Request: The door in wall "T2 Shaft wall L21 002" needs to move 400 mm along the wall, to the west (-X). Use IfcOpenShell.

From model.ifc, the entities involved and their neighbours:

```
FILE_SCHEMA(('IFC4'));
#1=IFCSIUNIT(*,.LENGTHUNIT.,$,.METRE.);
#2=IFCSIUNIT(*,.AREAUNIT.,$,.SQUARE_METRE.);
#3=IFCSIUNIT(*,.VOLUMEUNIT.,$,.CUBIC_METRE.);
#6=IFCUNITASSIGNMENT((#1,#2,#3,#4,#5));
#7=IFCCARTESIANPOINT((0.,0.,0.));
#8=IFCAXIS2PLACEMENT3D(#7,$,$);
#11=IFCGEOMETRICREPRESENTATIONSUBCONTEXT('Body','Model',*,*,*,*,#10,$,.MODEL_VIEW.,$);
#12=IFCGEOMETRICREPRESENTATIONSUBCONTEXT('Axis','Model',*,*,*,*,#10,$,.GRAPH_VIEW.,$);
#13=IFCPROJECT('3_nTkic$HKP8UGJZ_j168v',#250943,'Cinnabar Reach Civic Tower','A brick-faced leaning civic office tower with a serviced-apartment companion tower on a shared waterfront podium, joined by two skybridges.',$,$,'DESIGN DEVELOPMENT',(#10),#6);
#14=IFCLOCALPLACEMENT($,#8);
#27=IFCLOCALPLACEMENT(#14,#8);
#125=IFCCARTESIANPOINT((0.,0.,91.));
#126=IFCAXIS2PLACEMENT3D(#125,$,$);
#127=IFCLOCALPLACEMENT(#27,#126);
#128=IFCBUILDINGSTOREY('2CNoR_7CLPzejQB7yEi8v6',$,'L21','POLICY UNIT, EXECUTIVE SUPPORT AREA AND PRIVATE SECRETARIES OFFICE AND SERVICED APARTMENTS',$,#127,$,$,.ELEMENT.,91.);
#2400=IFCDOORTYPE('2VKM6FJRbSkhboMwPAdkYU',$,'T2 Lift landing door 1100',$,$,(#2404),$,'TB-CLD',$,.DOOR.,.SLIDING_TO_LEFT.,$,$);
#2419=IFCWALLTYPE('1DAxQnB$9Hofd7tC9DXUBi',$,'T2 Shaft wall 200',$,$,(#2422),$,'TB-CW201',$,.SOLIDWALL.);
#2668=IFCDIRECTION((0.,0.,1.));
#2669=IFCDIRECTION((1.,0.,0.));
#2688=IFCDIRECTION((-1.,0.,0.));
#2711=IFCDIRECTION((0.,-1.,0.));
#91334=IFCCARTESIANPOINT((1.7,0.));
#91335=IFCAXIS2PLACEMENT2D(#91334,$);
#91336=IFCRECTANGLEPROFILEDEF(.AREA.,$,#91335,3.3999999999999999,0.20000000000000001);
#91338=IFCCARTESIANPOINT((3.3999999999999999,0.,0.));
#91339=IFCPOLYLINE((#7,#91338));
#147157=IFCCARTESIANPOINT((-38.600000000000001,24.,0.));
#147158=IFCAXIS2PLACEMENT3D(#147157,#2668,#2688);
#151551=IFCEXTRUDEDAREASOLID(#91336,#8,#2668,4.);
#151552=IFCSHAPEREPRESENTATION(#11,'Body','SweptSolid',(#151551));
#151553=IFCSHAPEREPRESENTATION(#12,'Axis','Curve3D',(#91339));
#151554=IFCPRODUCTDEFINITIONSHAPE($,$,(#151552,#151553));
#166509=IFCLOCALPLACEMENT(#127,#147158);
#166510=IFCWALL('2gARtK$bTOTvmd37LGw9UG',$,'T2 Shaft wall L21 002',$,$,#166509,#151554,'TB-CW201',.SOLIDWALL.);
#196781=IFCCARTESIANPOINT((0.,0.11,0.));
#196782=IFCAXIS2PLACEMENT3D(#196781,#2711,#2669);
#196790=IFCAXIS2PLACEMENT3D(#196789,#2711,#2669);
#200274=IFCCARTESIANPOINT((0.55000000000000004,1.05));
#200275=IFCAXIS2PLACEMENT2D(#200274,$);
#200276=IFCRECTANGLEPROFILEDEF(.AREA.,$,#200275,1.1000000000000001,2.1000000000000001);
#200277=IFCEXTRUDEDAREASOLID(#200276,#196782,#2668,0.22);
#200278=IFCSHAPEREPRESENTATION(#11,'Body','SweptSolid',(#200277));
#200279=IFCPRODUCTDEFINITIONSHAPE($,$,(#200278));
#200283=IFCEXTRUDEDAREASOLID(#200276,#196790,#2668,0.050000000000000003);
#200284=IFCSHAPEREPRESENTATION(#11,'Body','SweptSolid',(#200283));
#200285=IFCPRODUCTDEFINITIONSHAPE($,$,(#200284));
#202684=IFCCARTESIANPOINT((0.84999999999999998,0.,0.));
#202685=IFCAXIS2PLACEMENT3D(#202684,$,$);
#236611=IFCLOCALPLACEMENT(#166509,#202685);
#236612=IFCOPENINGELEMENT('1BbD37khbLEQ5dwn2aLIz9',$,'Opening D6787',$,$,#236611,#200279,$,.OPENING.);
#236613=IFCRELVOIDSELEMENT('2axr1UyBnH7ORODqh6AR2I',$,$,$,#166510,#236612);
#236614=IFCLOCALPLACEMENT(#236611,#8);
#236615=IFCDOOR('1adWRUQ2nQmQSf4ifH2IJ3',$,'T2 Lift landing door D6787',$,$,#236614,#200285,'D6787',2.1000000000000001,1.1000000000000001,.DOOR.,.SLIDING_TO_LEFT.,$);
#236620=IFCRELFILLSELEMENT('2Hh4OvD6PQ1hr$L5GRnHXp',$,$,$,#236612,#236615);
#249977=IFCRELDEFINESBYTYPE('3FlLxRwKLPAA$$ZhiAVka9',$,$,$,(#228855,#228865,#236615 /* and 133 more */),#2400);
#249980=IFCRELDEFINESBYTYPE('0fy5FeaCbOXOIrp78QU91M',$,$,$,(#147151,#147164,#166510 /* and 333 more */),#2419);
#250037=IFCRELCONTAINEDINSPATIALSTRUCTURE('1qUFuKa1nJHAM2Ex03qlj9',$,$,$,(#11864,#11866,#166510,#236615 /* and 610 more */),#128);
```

```python
import ifcopenshell
import ifcopenshell.api.geometry
import ifcopenshell.util.placement
import ifcopenshell.util.unit

model = ifcopenshell.open("model.ifc")
unit_scale = ifcopenshell.util.unit.calculate_unit_scale(model)

door = model.by_guid("1adWRUQ2nQmQSf4ifH2IJ3")
opening = door.FillsVoids[0].RelatingOpeningElement
wall = opening.VoidsElements[0].RelatingBuildingElement

wall_matrix = ifcopenshell.util.placement.get_local_placement(wall.ObjectPlacement)
shift = wall_matrix[:3, 0] * 0.4 / unit_scale
before = ifcopenshell.util.placement.get_local_placement(door.ObjectPlacement)[:3, 3].copy()

# The door is placed relative to its opening, so it follows when the opening moves.
matrix = ifcopenshell.util.placement.get_local_placement(opening.ObjectPlacement)
matrix[:3, 3] += shift
ifcopenshell.api.geometry.edit_object_placement(
    model, product=opening, matrix=matrix, is_si=False, should_transform_children=True
)

after = ifcopenshell.util.placement.get_local_placement(door.ObjectPlacement)[:3, 3]
print("door moved by", (after - before).round(3) + 0.0)

model.write("model_v2.ifc")
```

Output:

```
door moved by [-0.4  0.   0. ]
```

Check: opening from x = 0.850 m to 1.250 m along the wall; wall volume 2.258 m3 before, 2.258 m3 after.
